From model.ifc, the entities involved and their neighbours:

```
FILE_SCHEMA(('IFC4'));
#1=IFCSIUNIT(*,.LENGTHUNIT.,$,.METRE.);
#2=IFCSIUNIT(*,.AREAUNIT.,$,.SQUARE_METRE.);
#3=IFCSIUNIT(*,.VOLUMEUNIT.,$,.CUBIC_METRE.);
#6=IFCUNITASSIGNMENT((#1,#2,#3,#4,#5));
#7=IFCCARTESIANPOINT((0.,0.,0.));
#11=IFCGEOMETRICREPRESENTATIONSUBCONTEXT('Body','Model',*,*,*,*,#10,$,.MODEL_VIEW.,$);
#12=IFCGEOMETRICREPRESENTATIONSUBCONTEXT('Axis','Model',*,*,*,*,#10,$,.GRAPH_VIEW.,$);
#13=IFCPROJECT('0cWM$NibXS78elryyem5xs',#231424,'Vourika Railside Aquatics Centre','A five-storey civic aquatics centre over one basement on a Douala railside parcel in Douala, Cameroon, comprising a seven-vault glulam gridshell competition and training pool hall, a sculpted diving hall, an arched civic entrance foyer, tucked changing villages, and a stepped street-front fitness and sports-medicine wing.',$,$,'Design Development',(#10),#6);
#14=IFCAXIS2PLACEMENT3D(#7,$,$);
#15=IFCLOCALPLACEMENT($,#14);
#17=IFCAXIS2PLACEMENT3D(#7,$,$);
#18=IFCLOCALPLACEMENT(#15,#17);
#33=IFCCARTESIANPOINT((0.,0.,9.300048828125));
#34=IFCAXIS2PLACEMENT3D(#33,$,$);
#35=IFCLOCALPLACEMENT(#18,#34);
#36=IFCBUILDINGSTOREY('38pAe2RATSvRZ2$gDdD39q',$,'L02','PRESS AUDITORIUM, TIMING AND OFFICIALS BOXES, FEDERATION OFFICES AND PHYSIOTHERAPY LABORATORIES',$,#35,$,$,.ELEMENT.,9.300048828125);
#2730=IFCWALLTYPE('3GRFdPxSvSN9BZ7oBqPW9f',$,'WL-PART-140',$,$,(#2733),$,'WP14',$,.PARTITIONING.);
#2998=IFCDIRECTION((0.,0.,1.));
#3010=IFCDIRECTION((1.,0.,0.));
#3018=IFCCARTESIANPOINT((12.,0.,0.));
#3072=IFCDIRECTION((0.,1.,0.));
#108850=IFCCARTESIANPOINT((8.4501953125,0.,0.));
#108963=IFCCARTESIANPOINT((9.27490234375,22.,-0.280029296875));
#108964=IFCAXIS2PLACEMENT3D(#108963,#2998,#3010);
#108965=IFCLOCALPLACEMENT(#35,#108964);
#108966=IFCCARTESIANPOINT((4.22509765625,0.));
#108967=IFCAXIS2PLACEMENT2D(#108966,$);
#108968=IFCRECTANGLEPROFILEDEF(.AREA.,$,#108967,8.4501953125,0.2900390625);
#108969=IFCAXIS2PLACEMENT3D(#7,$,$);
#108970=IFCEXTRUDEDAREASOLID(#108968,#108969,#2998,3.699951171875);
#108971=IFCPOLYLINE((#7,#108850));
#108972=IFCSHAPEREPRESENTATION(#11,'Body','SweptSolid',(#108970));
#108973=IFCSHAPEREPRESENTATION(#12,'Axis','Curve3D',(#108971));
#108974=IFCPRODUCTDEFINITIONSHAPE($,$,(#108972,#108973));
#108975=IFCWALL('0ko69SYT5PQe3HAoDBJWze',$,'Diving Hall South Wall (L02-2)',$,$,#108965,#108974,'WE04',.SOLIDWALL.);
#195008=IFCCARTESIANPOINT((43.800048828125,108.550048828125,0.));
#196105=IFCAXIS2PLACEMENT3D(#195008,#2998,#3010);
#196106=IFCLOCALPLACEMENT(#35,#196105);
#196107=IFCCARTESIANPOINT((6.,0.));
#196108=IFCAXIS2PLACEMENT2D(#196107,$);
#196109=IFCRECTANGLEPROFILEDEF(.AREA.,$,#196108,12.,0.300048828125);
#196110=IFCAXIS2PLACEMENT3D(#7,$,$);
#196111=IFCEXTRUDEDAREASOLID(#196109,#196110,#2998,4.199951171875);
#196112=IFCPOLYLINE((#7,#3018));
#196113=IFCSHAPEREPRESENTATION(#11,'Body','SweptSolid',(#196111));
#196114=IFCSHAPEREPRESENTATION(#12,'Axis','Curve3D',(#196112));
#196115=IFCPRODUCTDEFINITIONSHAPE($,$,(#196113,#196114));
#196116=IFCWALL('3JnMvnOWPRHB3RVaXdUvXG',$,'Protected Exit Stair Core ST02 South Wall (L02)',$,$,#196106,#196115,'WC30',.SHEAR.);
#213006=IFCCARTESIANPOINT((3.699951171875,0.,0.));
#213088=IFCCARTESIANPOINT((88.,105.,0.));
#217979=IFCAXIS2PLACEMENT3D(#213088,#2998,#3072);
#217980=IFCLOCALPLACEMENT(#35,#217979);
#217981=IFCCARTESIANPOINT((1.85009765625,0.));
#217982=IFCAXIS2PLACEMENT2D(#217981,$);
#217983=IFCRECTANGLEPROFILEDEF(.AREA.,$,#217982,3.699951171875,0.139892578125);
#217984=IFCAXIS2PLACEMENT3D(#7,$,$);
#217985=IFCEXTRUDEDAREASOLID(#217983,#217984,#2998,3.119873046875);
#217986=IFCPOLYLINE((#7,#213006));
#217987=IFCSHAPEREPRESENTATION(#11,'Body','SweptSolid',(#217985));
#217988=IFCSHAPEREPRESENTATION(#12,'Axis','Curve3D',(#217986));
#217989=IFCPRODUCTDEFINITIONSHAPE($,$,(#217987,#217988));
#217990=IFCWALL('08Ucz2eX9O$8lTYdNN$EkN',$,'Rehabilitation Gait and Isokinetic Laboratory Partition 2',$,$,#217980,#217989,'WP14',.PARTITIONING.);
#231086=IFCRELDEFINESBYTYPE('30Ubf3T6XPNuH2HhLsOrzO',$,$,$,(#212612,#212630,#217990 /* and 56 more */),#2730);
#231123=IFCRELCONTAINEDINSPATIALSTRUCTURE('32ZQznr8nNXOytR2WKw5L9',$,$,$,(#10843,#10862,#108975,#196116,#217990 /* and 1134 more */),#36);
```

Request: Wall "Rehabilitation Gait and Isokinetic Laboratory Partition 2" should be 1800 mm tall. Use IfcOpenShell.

```python
import ifcopenshell
import ifcopenshell.geom
import ifcopenshell.util.representation
import ifcopenshell.util.shape
import ifcopenshell.util.unit

model = ifcopenshell.open("model.ifc")
unit_scale = ifcopenshell.util.unit.calculate_unit_scale(model)
settings = ifcopenshell.geom.settings()


def volume(element):
    """Net volume in cubic metres, openings subtracted."""
    shape = ifcopenshell.geom.create_shape(settings, element)
    return ifcopenshell.util.shape.get_volume(shape.geometry)


wall = model.by_guid("08Ucz2eX9O$8lTYdNN$EkN")
before = volume(wall)

body = ifcopenshell.util.representation.get_representation(wall, "Model", "Body")
solid = body.Items[0]
old_height = solid.Depth
solid.Depth = 1.8 / unit_scale
after = volume(wall)

print(f"height {old_height:g} -> {solid.Depth:g}, volume {before:.3f} -> {after:.3f} m3")

model.write("model_updated.ifc")
```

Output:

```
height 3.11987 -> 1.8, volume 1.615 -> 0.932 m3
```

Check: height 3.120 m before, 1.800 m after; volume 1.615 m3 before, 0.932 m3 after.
